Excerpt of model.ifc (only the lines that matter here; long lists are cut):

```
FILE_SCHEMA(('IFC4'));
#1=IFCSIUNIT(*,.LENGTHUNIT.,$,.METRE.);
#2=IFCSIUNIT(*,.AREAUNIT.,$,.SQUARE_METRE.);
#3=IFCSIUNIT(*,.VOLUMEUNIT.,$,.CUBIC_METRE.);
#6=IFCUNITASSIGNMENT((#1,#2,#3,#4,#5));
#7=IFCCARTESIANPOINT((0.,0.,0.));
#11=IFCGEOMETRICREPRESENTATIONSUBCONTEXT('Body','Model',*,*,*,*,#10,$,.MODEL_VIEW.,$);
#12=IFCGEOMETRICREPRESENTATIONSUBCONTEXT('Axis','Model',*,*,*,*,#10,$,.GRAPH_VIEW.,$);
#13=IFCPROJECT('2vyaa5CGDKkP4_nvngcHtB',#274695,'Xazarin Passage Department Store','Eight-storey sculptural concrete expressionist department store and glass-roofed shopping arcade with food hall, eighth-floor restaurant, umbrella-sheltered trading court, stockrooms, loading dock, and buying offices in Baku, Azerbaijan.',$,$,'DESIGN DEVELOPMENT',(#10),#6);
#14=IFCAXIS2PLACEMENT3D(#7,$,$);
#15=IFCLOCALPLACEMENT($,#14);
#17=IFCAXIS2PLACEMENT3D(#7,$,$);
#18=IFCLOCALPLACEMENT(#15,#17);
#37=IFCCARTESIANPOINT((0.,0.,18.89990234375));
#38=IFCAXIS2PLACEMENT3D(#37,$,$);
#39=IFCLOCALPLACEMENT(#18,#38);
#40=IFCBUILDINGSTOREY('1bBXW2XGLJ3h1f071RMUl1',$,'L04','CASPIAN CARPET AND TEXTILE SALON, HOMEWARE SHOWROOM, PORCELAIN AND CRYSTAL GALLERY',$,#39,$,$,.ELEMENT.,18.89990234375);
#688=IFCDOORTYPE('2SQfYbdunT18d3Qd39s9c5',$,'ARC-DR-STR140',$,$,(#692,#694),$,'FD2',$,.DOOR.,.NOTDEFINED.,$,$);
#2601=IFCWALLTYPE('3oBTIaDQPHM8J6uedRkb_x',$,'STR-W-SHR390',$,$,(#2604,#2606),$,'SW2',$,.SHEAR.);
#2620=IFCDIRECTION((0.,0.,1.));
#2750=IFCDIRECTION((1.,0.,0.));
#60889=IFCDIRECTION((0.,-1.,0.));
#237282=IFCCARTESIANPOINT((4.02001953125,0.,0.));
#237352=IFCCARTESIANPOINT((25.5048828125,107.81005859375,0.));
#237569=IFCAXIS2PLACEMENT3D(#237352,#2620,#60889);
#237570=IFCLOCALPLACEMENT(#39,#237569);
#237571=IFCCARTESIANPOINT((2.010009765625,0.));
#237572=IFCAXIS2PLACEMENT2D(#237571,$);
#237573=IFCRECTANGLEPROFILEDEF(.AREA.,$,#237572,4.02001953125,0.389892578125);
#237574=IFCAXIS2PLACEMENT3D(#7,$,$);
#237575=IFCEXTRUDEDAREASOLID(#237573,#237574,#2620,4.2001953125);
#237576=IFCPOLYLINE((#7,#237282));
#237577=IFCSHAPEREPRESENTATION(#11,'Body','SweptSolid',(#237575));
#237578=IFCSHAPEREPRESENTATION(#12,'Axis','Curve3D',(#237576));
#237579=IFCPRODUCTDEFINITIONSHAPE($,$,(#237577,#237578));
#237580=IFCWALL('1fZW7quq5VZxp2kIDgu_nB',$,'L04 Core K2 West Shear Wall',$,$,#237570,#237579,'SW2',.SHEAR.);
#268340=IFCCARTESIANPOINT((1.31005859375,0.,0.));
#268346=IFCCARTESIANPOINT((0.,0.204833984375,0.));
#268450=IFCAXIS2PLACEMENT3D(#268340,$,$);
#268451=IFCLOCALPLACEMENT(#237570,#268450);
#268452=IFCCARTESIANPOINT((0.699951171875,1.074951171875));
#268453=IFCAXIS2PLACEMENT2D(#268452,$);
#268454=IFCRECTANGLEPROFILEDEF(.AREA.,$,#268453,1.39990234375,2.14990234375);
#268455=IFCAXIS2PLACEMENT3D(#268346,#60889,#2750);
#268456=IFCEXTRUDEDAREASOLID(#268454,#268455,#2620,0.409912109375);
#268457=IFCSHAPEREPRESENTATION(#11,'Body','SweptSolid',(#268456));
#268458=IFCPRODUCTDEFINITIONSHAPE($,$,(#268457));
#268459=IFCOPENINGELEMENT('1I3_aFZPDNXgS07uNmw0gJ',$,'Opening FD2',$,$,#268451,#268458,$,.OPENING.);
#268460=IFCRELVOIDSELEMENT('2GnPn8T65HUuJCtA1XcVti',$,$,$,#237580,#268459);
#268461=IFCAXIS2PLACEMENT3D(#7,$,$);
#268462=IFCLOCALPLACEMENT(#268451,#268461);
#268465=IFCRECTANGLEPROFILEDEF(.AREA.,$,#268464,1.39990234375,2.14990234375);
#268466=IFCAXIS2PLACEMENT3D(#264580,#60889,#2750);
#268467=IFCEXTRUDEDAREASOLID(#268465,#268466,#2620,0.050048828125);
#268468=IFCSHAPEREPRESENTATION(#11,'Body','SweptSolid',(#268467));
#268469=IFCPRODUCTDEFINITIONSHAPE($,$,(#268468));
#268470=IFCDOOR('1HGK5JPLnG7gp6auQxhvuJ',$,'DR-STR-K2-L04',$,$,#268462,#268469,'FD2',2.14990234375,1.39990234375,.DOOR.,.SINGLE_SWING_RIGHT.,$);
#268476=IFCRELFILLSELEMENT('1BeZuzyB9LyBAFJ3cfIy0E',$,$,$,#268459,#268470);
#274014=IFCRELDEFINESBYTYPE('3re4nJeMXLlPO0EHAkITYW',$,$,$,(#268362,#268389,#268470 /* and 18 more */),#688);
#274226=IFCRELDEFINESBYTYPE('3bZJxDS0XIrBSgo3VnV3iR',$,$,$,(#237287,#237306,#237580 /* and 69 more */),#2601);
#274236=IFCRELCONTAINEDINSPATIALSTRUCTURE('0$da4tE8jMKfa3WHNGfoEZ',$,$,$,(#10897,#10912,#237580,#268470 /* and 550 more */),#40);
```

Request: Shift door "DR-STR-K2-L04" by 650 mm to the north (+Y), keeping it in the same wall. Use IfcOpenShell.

```python
import ifcopenshell
import ifcopenshell.api.geometry
import ifcopenshell.util.placement

model = ifcopenshell.open("model.ifc")

door = model.by_id(268470)
opening = door.FillsVoids[0].RelatingOpeningElement
wall = opening.VoidsElements[0].RelatingBuildingElement

wall_matrix = ifcopenshell.util.placement.get_local_placement(wall.ObjectPlacement)
shift = wall_matrix[:3, 0] * -0.65
before = ifcopenshell.util.placement.get_local_placement(door.ObjectPlacement)[:3, 3].copy()

# The door is placed relative to its opening, so it follows when the opening moves.
matrix = ifcopenshell.util.placement.get_local_placement(opening.ObjectPlacement)
matrix[:3, 3] += shift
ifcopenshell.api.geometry.edit_object_placement(
    model, product=opening, matrix=matrix, is_si=False, should_transform_children=True
)

after = ifcopenshell.util.placement.get_local_placement(door.ObjectPlacement)[:3, 3]
print("door moved by", (after - before).round(3) + 0.0)

model.write("model-out.ifc")
```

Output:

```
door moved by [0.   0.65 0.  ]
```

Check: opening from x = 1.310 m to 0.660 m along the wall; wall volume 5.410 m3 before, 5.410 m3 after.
